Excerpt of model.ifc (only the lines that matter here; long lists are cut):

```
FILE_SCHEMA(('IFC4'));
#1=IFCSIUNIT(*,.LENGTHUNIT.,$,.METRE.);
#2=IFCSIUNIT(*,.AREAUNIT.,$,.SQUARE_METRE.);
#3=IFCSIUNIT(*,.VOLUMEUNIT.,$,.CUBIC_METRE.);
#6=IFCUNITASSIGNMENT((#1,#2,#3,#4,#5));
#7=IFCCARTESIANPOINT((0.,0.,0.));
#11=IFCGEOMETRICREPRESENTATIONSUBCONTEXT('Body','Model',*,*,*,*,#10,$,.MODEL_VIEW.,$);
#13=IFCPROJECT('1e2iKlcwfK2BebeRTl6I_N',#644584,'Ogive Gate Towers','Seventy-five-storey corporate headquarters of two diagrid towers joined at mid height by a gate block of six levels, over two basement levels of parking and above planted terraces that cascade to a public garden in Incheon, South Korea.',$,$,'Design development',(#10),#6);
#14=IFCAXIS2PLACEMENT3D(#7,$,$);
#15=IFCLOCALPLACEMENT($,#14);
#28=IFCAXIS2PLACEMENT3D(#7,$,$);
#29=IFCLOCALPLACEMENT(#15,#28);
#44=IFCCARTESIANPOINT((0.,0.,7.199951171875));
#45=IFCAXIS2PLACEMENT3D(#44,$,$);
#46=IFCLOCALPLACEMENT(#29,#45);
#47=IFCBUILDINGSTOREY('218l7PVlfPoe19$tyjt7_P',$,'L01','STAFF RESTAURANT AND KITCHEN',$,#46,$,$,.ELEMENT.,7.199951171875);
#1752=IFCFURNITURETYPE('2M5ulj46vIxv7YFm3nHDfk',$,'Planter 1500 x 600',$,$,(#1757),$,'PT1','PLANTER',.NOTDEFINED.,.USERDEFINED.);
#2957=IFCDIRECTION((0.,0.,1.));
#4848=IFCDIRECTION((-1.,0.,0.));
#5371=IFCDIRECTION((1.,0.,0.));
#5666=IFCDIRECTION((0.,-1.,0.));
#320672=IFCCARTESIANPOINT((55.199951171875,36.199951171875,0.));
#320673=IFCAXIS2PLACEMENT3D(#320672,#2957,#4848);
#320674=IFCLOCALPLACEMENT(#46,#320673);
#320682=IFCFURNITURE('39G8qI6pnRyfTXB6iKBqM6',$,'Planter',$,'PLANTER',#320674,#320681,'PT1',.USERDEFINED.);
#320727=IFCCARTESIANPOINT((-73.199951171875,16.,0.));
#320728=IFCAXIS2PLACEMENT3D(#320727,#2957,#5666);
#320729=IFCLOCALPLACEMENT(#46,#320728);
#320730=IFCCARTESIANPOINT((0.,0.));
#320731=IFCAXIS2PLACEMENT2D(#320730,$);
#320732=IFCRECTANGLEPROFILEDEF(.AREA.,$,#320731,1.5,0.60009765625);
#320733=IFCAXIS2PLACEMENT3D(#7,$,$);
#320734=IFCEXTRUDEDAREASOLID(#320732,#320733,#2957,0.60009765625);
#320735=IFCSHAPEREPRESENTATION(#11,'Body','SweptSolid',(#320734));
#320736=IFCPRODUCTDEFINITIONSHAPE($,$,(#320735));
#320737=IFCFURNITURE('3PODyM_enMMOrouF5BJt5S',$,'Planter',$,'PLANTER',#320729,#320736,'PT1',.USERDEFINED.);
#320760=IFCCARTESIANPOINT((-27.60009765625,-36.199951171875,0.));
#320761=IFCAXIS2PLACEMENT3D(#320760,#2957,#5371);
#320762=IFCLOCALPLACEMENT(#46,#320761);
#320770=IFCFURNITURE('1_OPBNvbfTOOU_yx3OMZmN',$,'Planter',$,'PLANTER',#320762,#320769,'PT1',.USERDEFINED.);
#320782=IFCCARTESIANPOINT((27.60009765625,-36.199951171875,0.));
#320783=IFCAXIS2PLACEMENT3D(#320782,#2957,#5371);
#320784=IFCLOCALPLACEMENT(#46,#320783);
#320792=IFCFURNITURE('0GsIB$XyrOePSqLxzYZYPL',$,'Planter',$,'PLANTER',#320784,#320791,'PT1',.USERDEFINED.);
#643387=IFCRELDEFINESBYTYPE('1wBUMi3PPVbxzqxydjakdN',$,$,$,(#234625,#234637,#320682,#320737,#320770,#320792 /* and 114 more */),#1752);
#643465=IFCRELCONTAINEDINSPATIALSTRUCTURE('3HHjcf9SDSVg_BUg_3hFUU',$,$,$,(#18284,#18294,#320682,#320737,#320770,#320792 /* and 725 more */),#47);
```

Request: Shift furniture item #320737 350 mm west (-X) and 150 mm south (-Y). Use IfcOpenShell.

```python
import ifcopenshell
import ifcopenshell.api.geometry
import ifcopenshell.util.placement
import ifcopenshell.util.unit

model = ifcopenshell.open("model.ifc")
unit_scale = ifcopenshell.util.unit.calculate_unit_scale(model)

item = model.by_id(320737)
matrix = ifcopenshell.util.placement.get_local_placement(item.ObjectPlacement)
matrix[0, 3] -= 0.35 / unit_scale
matrix[1, 3] -= 0.15 / unit_scale
ifcopenshell.api.geometry.edit_object_placement(model, product=item, matrix=matrix, is_si=False)

print(ifcopenshell.util.placement.get_local_placement(item.ObjectPlacement).round(3) + 0.0)

model.write("model_edited.ifc")
```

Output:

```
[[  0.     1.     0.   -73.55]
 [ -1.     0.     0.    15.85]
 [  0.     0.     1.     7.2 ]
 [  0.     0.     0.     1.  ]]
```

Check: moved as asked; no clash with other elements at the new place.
